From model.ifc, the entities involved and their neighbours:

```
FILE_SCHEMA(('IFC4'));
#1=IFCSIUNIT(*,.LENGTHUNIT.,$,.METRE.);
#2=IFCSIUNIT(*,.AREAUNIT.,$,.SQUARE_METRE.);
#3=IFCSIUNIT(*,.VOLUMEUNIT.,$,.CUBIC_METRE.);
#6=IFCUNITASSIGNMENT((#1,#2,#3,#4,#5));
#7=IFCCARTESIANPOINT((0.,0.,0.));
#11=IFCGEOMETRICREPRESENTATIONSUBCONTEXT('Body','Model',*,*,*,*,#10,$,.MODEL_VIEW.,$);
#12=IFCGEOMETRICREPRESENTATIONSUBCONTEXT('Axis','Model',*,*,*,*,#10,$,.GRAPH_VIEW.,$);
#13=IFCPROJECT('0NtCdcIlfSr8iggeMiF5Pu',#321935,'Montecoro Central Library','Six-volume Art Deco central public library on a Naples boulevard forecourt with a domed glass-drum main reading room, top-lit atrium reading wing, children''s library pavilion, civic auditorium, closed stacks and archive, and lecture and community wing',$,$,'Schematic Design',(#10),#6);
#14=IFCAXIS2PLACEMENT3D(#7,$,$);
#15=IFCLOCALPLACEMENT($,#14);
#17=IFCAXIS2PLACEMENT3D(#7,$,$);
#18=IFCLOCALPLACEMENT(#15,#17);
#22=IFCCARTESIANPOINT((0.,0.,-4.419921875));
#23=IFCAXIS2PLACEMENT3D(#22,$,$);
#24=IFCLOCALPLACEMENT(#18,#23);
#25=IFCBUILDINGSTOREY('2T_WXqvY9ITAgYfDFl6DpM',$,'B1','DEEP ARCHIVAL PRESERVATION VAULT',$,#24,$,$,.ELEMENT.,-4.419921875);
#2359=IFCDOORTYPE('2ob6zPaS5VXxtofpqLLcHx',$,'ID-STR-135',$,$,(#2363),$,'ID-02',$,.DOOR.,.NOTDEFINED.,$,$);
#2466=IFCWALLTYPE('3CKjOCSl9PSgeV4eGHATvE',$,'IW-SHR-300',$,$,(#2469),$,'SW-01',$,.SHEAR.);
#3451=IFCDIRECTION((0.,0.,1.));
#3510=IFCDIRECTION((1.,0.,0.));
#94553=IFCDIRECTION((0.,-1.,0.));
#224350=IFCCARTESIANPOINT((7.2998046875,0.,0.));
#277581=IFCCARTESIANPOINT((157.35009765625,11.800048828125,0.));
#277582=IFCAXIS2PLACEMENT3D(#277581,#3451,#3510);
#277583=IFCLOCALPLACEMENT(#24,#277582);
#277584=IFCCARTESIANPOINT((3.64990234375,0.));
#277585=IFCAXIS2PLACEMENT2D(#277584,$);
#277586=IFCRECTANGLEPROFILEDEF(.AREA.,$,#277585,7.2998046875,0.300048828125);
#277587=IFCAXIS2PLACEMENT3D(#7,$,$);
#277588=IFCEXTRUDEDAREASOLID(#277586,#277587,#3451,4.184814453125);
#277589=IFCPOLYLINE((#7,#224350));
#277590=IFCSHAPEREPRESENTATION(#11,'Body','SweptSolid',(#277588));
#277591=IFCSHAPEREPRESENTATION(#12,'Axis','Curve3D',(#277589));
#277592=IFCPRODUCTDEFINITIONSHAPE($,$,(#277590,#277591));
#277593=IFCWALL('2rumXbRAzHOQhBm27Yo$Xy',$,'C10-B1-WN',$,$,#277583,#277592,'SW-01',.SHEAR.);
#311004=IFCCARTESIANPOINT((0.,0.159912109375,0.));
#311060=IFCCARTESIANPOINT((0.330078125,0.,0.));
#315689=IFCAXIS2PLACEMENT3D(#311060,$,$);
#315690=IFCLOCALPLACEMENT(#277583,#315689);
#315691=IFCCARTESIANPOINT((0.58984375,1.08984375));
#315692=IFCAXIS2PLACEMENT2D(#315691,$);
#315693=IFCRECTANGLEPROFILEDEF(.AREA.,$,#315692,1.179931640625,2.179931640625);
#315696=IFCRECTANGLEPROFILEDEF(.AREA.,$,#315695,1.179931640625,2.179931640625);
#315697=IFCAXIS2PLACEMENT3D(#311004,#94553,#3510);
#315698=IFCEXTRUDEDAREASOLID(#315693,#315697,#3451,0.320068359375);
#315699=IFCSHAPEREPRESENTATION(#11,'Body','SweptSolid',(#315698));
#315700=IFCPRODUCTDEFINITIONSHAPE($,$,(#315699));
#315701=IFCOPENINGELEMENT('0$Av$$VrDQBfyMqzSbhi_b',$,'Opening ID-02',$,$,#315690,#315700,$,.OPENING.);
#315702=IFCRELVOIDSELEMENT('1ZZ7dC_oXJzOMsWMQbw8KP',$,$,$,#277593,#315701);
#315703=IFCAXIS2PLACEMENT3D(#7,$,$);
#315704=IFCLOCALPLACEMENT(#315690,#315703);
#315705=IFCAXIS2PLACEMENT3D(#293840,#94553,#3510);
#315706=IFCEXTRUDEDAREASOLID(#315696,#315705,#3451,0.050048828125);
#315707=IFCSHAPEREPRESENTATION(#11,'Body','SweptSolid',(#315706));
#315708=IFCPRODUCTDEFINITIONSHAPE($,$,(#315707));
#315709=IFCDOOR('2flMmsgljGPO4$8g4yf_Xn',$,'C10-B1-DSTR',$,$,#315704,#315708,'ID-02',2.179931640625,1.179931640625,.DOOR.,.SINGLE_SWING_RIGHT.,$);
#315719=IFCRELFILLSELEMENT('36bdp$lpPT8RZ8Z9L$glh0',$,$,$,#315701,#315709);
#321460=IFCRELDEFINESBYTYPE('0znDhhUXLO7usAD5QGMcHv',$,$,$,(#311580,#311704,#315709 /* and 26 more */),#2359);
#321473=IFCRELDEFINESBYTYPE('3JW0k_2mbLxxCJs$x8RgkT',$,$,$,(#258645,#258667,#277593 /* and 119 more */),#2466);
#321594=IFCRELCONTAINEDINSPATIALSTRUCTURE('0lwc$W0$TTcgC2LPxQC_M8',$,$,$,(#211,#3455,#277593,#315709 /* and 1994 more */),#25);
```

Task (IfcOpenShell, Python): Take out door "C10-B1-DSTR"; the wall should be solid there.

```python
import ifcopenshell
import ifcopenshell.api.feature
import ifcopenshell.api.root
import ifcopenshell.geom
import ifcopenshell.util.shape

model = ifcopenshell.open("model.ifc")
settings = ifcopenshell.geom.settings()


def volume(element):
    """Net volume in cubic metres, openings subtracted."""
    shape = ifcopenshell.geom.create_shape(settings, element)
    return ifcopenshell.util.shape.get_volume(shape.geometry)


door = model.by_guid("2flMmsgljGPO4$8g4yf_Xn")
opening = door.FillsVoids[0].RelatingOpeningElement
wall = opening.VoidsElements[0].RelatingBuildingElement
before = volume(wall)

ifcopenshell.api.root.remove_product(model, product=door)
ifcopenshell.api.feature.remove_feature(model, feature=opening)

after = volume(wall)

print(f"wall volume {before:.3f} -> {after:.3f} m3")

model.write("model_updated.ifc")
```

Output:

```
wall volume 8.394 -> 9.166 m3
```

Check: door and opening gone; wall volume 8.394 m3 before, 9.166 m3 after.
